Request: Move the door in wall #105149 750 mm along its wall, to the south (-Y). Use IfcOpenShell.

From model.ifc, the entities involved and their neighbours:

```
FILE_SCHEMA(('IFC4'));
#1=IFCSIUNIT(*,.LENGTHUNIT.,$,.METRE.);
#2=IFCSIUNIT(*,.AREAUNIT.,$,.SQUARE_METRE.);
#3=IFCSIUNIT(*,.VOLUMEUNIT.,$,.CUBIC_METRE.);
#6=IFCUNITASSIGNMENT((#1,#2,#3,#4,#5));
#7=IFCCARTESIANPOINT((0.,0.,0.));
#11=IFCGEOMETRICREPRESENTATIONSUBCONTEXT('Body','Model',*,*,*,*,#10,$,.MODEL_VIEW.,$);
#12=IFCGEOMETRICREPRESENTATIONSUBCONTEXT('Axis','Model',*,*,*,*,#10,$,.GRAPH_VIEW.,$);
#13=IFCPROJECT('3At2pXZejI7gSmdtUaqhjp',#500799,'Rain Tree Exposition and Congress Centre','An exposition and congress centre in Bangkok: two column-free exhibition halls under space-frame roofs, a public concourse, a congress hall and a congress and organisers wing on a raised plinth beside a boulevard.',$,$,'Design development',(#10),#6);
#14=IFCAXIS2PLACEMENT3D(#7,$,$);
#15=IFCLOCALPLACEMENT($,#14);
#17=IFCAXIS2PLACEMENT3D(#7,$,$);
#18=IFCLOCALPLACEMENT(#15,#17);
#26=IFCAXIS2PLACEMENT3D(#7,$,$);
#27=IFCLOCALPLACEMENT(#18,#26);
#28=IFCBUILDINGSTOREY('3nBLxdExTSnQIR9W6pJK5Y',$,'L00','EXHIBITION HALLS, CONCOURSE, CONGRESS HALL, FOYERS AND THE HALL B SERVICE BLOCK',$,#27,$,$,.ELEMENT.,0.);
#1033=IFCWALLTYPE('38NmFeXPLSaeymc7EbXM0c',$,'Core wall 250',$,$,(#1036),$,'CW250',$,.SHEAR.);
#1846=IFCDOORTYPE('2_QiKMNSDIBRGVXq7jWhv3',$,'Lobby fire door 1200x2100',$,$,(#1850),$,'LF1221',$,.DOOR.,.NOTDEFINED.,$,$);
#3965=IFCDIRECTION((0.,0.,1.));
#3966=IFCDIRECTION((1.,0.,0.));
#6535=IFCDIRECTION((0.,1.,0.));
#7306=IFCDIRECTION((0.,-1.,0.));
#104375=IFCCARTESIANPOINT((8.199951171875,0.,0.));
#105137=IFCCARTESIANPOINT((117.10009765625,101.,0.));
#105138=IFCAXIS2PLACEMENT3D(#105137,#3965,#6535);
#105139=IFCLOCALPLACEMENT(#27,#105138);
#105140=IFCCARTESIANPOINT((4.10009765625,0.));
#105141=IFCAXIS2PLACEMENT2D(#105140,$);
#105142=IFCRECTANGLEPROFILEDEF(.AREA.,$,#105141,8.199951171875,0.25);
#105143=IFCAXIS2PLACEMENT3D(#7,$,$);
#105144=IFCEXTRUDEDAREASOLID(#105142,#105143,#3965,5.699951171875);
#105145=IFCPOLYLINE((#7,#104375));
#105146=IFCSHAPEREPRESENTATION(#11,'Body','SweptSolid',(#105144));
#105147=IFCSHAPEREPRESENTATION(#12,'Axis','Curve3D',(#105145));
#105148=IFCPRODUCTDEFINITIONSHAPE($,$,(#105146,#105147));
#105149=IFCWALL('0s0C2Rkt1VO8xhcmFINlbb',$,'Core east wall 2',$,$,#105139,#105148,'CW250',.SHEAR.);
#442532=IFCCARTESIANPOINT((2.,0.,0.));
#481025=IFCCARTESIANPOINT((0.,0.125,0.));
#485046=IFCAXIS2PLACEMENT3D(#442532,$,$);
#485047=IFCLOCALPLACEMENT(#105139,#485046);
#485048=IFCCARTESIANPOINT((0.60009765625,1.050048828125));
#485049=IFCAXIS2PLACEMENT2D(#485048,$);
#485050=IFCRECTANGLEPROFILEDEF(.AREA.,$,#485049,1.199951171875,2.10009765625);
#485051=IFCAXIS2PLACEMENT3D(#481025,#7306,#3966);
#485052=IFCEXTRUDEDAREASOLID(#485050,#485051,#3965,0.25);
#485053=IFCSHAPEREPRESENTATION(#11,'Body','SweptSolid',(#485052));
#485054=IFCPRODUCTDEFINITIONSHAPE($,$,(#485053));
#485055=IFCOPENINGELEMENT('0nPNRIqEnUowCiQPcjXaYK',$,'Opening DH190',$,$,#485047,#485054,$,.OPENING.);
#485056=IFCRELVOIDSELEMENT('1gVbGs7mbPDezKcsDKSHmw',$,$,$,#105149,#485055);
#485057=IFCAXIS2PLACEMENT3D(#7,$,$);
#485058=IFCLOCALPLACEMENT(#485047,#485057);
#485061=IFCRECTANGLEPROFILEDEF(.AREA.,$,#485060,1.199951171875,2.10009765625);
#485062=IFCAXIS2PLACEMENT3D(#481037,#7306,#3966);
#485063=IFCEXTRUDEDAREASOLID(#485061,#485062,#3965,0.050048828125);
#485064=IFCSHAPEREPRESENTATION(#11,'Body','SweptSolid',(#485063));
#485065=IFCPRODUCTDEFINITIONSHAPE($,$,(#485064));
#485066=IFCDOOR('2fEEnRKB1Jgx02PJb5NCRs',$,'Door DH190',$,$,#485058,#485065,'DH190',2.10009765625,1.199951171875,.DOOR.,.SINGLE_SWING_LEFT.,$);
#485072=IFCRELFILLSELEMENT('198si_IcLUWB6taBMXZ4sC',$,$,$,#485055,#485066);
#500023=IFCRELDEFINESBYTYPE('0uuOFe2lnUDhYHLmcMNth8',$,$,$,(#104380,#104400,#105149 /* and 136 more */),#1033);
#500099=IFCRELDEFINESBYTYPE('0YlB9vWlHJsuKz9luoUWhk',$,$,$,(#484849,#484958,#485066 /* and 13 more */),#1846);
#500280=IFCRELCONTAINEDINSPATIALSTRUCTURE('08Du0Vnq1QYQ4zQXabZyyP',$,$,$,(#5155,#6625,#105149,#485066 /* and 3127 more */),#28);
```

```python
import ifcopenshell
import ifcopenshell.api.geometry
import ifcopenshell.util.placement
import ifcopenshell.util.unit

model = ifcopenshell.open("model.ifc")
unit_scale = ifcopenshell.util.unit.calculate_unit_scale(model)

door = model.by_guid("2fEEnRKB1Jgx02PJb5NCRs")
opening = door.FillsVoids[0].RelatingOpeningElement
wall = opening.VoidsElements[0].RelatingBuildingElement

wall_matrix = ifcopenshell.util.placement.get_local_placement(wall.ObjectPlacement)
shift = wall_matrix[:3, 0] * -0.75 / unit_scale
before = ifcopenshell.util.placement.get_local_placement(door.ObjectPlacement)[:3, 3].copy()

# The door is placed relative to its opening, so it follows when the opening moves.
matrix = ifcopenshell.util.placement.get_local_placement(opening.ObjectPlacement)
matrix[:3, 3] += shift
ifcopenshell.api.geometry.edit_object_placement(
    model, product=opening, matrix=matrix, is_si=False, should_transform_children=True
)

after = ifcopenshell.util.placement.get_local_placement(door.ObjectPlacement)[:3, 3]
print("door moved by", (after - before).round(3) + 0.0)

model.write("model_updated.ifc")
```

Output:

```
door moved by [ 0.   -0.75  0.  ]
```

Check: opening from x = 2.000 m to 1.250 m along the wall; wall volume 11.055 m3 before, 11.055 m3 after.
